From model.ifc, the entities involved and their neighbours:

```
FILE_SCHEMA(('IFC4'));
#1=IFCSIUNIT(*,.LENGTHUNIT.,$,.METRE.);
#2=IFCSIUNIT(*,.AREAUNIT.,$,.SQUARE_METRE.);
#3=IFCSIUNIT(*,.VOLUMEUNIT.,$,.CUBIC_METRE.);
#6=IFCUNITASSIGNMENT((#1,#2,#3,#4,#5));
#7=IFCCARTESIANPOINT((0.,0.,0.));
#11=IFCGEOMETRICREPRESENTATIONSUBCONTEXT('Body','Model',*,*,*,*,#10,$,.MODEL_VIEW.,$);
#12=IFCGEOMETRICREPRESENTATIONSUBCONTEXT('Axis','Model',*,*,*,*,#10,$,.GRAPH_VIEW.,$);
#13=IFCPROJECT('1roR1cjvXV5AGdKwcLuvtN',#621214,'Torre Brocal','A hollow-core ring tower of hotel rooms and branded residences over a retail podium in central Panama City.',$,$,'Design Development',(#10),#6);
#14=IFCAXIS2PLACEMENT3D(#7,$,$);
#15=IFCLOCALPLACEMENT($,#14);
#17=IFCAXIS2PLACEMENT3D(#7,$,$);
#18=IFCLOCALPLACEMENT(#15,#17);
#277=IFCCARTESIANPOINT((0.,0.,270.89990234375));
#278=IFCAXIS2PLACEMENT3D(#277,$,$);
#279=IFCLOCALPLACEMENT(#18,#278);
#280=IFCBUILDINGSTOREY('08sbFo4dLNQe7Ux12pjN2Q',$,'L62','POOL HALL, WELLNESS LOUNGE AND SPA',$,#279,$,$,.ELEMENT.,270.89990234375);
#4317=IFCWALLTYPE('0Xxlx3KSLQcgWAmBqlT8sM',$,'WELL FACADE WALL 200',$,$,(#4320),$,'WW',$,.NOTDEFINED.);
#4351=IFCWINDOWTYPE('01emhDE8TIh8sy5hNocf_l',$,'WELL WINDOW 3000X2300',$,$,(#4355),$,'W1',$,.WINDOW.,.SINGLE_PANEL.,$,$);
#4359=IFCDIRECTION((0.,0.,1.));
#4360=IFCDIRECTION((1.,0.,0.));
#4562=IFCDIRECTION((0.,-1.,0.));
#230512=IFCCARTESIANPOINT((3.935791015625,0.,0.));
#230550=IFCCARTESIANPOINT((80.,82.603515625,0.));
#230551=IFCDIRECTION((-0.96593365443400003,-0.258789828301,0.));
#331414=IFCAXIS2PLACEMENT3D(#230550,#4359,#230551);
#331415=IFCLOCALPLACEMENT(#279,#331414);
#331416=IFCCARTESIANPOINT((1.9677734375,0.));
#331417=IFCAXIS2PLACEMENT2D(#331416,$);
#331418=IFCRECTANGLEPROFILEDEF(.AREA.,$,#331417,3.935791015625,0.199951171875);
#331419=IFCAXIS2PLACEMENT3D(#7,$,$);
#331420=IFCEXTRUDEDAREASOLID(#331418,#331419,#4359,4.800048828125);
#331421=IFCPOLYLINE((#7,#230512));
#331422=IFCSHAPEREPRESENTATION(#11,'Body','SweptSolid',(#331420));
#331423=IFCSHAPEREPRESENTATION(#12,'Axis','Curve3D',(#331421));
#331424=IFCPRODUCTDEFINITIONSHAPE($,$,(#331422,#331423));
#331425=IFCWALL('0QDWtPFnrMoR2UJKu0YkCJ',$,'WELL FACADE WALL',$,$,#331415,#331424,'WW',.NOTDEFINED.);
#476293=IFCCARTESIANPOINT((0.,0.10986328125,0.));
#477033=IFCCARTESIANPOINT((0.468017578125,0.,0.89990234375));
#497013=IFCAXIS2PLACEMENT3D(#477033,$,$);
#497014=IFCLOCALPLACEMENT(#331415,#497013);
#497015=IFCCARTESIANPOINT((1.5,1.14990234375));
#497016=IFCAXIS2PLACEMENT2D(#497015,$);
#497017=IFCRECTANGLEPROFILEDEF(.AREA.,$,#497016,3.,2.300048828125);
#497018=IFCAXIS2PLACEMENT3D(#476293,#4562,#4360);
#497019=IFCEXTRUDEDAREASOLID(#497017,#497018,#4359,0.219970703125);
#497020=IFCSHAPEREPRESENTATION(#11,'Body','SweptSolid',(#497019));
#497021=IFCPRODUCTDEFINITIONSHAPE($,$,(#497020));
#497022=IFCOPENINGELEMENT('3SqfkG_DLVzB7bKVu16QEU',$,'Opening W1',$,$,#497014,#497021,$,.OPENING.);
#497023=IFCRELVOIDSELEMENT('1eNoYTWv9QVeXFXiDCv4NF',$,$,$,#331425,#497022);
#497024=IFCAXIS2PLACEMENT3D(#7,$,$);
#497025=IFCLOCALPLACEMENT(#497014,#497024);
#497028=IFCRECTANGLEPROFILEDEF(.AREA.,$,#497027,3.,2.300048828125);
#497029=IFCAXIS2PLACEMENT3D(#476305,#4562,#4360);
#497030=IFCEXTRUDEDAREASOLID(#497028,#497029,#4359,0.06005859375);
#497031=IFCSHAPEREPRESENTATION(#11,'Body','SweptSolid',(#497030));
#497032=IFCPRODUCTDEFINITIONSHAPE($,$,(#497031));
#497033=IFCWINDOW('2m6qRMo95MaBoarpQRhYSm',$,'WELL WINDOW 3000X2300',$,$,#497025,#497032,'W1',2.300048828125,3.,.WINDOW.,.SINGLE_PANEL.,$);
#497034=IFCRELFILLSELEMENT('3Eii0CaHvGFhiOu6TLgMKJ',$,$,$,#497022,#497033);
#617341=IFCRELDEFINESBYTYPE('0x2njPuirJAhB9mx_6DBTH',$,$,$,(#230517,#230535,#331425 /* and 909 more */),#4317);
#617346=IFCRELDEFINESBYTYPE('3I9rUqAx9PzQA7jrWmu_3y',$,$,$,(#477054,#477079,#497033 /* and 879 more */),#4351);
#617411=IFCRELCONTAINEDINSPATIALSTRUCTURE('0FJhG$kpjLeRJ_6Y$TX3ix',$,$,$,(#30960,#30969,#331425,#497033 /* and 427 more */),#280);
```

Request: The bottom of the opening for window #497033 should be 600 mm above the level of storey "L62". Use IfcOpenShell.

```python
import numpy as np
import ifcopenshell
import ifcopenshell.api.geometry
import ifcopenshell.geom
import ifcopenshell.util.element
import ifcopenshell.util.placement
import ifcopenshell.util.shape
import ifcopenshell.util.unit

model = ifcopenshell.open("model.ifc")
unit_scale = ifcopenshell.util.unit.calculate_unit_scale(model)

window = model.by_id(497033)
opening = window.FillsVoids[0].RelatingOpeningElement
storey = ifcopenshell.util.element.get_container(window, ifc_class="IfcBuildingStorey")
level = ifcopenshell.util.placement.get_local_placement(storey.ObjectPlacement)[2, 3]

# The opening's origin need not be at the sill, so measure its lowest point.
shape = ifcopenshell.geom.create_shape(ifcopenshell.geom.settings(), opening)
bottom = ifcopenshell.util.shape.get_shape_bottom_elevation(shape, shape.geometry) / unit_scale
dz = level + 0.6 / unit_scale - bottom

shift = np.array([0.0, 0.0, dz])
# The window is placed relative to its opening, so it follows when the opening moves.
matrix = ifcopenshell.util.placement.get_local_placement(opening.ObjectPlacement)
matrix[:3, 3] += shift
ifcopenshell.api.geometry.edit_object_placement(
    model, product=opening, matrix=matrix, is_si=False, should_transform_children=True
)

print(f"moved by {dz * unit_scale:+.3f} m")

model.write("model-out.ifc")
```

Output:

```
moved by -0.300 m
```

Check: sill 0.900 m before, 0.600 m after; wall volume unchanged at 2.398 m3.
